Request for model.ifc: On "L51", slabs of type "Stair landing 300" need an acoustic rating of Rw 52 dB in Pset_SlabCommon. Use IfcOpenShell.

First a look at what the model holds.

```python
import ifcopenshell
import ifcopenshell.util.element

model = ifcopenshell.open("model.ifc")
print(model.schema)
storey = next(s for s in model.by_type("IfcBuildingStorey") if s.Name == "L51")
slabs = [e for e in ifcopenshell.util.element.get_decomposition(storey) if e.is_a("IfcSlab")]
seen = {}
for e in slabs:
    element_type = ifcopenshell.util.element.get_type(e)
    key = (element_type.Name if element_type != e and element_type else None, ifcopenshell.util.element.get_pset(e, "Pset_SlabCommon", "AcousticRating"))
    seen[key] = seen.get(key, 0) + 1
for (name, value), count in sorted(seen.items(), key=str):
    print(count, "x", name, "|", value)
```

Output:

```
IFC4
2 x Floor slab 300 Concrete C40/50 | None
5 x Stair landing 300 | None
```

```python
import ifcopenshell
import ifcopenshell.api.pset
import ifcopenshell.util.element

model = ifcopenshell.open("model.ifc")

storey = next(s for s in model.by_type("IfcBuildingStorey") if s.Name == "L51")
slabs = [e for e in ifcopenshell.util.element.get_decomposition(storey) if e.is_a("IfcSlab")]

count = 0
for e in slabs:
    element_type = ifcopenshell.util.element.get_type(e)
    if element_type in (None, e) or element_type.Name != "Stair landing 300":
        continue
    found = ifcopenshell.util.element.get_pset(e, "Pset_SlabCommon", should_inherit=False)
    if found:
        pset = model.by_id(found["id"])
        if len(ifcopenshell.util.element.get_elements_by_pset(pset)) > 1:
            pset = ifcopenshell.api.pset.unshare_pset(model, products=[e], pset=pset)[0]
    else:
        pset = ifcopenshell.api.pset.add_pset(model, product=e, name="Pset_SlabCommon")
    ifcopenshell.api.pset.edit_pset(model, pset=pset, properties={"AcousticRating": "Rw 52 dB"})
    count += 1

print(count, "slabs updated")

model.write("model-out.ifc")
```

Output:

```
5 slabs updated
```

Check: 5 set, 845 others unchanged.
